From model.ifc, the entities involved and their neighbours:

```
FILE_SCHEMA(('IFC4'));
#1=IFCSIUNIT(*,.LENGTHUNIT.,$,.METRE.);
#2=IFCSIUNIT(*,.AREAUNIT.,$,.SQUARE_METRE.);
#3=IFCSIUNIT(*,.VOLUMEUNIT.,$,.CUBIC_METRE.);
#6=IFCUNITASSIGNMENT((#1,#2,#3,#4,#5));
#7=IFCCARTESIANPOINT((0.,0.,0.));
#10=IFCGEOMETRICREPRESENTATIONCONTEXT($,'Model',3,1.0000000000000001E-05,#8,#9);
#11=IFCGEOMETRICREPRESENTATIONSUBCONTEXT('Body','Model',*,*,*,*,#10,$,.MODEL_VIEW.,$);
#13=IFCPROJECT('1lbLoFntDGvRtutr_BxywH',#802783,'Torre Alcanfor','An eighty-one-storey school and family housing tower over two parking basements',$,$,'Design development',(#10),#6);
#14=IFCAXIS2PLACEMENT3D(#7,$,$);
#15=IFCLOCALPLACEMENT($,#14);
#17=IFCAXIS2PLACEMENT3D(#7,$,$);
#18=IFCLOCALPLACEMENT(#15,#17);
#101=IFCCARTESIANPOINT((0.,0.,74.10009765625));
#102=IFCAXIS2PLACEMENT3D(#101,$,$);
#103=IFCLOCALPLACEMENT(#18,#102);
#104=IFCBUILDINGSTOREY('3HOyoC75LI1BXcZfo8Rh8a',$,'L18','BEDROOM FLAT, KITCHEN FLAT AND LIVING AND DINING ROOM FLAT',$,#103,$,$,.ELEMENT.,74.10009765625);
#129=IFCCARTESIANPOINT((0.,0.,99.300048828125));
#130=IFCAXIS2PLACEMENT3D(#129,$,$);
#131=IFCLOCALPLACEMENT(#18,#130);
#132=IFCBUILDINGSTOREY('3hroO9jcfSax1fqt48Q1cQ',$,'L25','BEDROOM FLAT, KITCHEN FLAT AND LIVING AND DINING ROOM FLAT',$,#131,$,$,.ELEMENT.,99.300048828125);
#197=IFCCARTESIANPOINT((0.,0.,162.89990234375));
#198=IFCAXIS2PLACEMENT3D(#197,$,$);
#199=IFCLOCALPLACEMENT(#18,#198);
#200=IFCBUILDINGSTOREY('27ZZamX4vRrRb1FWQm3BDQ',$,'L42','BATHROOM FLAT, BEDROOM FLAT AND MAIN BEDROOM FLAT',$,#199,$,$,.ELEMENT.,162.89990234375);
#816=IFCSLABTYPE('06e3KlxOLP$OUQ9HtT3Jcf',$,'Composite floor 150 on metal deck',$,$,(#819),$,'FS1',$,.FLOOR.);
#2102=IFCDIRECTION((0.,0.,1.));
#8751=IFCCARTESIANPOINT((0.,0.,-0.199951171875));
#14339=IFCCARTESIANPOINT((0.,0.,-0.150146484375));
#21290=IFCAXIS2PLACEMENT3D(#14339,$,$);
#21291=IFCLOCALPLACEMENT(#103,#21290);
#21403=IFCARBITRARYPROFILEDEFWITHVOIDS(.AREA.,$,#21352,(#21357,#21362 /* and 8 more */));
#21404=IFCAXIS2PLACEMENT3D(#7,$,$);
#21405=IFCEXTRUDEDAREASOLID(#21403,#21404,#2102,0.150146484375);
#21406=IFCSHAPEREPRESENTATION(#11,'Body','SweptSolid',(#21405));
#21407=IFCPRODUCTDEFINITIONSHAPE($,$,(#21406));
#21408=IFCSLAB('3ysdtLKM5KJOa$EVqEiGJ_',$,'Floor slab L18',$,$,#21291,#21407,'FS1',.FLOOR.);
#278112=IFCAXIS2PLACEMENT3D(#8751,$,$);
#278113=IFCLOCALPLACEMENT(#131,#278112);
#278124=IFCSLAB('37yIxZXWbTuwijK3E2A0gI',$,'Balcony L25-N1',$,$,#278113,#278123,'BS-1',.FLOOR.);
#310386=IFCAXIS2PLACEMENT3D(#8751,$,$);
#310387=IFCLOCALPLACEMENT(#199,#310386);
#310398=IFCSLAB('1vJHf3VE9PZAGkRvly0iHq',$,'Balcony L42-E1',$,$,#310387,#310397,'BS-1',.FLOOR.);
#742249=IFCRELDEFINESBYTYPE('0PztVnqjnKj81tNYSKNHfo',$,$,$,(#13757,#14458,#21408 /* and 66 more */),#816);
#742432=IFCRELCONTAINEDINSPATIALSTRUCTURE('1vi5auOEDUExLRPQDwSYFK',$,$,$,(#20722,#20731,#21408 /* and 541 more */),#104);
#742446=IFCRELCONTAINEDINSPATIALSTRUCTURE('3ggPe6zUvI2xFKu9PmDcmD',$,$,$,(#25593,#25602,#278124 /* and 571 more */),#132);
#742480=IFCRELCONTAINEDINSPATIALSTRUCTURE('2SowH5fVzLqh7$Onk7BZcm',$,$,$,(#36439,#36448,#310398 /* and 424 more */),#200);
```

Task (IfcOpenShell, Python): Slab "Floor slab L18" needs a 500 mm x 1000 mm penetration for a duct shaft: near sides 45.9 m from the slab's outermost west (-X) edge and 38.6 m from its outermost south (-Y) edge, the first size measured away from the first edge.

```python
import numpy as np
import ifcopenshell
import ifcopenshell.api.feature
import ifcopenshell.api.geometry
import ifcopenshell.api.root
import ifcopenshell.geom
import ifcopenshell.util.placement
import ifcopenshell.util.representation
import ifcopenshell.util.shape
import ifcopenshell.util.unit

model = ifcopenshell.open("model.ifc")
unit_scale = ifcopenshell.util.unit.calculate_unit_scale(model)
settings = ifcopenshell.geom.settings()


def volume(element):
    """Net volume in cubic metres, openings subtracted."""
    shape = ifcopenshell.geom.create_shape(settings, element)
    return ifcopenshell.util.shape.get_volume(shape.geometry)


slab = model.by_guid("3ysdtLKM5KJOa$EVqEiGJ_")
before = volume(slab)

# Extent in the slab's own axes, in metres. The edges named are its -X and -Y sides.
slab_shape = ifcopenshell.geom.create_shape(settings, slab)
vertices = ifcopenshell.util.shape.get_vertices(slab_shape.geometry)
x_min, y_min, bottom = vertices.min(axis=0)
top = vertices[:, 2].max()

opening = ifcopenshell.api.root.create_entity(model, ifc_class="IfcOpeningElement", name="Duct shaft opening", predefined_type="OPENING")
context = ifcopenshell.util.representation.get_context(model, "Model", "Body", "MODEL_VIEW")
width, depth = 0.5, 1
outline = [(0.0, 0.0), (width, 0.0), (width, depth), (0.0, depth), (0.0, 0.0)]
# Overshoot both faces by 50 mm so the cut is clean.
shape = ifcopenshell.api.geometry.add_slab_representation(
    model, context=context, depth=top - bottom + 0.1, polyline=outline
)
ifcopenshell.api.geometry.assign_representation(model, product=opening, representation=shape)

matrix = ifcopenshell.util.placement.get_local_placement(slab.ObjectPlacement)
matrix[:, 3] = matrix @ np.append(np.array([x_min + 45.9, y_min + 38.6, bottom - 0.05]) / unit_scale, 1.0)
ifcopenshell.api.geometry.edit_object_placement(model, product=opening, matrix=matrix, is_si=False)
ifcopenshell.api.feature.add_feature(model, feature=opening, element=slab)

after = volume(slab)

print(f"slab volume {before:.3f} -> {after:.3f} m3")

model.write("model_v2.ifc")
```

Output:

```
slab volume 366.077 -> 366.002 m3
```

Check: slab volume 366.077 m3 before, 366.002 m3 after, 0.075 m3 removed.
